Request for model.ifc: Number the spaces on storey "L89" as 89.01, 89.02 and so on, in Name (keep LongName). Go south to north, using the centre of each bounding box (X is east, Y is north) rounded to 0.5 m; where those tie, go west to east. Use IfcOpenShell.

First a look at what the model holds.

```python
import ifcopenshell
import ifcopenshell.util.element
import ifcopenshell.util.placement

model = ifcopenshell.open("model.ifc")
print(model.schema)
storey = next(s for s in model.by_type("IfcBuildingStorey") if s.Name == "L89")
spaces = [e for e in ifcopenshell.util.element.get_decomposition(storey) if e.is_a("IfcSpace")]
for e in sorted(spaces, key=lambda e: e.id()):
    origin = ifcopenshell.util.placement.get_local_placement(e.ObjectPlacement)[:3, 3]
    print(e.id(), e.Name, e.LongName, origin.round(2) + 0.0, sep=" | ")
```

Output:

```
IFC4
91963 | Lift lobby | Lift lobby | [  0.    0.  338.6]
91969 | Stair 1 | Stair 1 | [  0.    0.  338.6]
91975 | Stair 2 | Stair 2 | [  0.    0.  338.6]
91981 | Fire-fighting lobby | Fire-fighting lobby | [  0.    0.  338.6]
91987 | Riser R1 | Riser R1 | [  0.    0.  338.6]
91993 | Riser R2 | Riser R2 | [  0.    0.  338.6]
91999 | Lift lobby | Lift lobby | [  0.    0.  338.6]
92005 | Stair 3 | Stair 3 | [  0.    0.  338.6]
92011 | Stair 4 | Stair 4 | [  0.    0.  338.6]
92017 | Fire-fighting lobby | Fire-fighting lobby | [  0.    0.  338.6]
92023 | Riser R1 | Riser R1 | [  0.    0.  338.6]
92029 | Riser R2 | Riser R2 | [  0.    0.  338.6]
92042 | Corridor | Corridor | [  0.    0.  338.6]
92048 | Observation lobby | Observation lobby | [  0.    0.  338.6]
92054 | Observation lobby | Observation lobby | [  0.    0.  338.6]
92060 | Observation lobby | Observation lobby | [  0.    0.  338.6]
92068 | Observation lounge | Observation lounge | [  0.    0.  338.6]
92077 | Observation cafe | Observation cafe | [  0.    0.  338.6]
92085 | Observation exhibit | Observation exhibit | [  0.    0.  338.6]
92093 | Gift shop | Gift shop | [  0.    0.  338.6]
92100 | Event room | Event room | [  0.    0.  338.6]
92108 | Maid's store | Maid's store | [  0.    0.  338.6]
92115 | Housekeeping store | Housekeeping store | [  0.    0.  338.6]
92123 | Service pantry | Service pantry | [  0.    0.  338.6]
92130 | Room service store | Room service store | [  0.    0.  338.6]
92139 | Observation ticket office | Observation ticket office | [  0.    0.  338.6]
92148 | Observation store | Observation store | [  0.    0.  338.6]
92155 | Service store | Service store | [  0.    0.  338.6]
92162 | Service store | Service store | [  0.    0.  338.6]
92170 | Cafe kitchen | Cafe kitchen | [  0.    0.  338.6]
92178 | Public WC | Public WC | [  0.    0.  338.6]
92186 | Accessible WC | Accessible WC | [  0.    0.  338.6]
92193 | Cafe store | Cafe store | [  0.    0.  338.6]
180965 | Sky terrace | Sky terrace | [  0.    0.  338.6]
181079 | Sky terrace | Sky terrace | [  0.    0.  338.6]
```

```python
import ifcopenshell
import ifcopenshell.geom
import ifcopenshell.util.element
import ifcopenshell.util.shape

model = ifcopenshell.open("model.ifc")
settings = ifcopenshell.geom.settings()
settings.set("use-world-coords", True)


def centre(element):
    shape = ifcopenshell.geom.create_shape(settings, element)
    return ifcopenshell.util.shape.get_bbox_centroid(shape.geometry)


storey = next(s for s in model.by_type("IfcBuildingStorey") if s.Name == "L89")
spaces = [e for e in ifcopenshell.util.element.get_decomposition(storey) if e.is_a("IfcSpace")]

# Insertion points can sit at a corner or the storey origin, so sort by the geometry (in metres).
centres = {e: centre(e) for e in spaces}
spaces.sort(key=lambda e: (round(centres[e][1] / 0.5), centres[e][0]))

for i, e in enumerate(spaces, start=1):
    number = f"89.{i:02d}"
    e.Name = number
    print(e.id(), number)

model.write("model-out.ifc")
```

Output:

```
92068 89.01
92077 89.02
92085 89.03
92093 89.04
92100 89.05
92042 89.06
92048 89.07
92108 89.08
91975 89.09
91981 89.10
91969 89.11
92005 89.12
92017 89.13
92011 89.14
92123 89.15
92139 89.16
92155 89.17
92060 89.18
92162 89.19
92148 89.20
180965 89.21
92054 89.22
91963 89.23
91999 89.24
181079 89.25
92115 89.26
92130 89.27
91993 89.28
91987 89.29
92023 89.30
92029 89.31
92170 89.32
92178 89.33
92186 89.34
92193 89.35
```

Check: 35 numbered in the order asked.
